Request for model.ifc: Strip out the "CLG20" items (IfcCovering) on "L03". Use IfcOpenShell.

First a look at what the model holds.

```python
import ifcopenshell
import ifcopenshell.util.element

model = ifcopenshell.open("model.ifc")
print(model.schema)
storey = next(s for s in model.by_type("IfcBuildingStorey") if s.Name == "L03")
coverings = [e for e in ifcopenshell.util.element.get_decomposition(storey) if e.is_a("IfcCovering")]
seen = {}
for e in coverings:
    element_type = ifcopenshell.util.element.get_type(e)
    name = element_type.Name if element_type not in (None, e) else None
    seen[name] = seen.get(name, 0) + 1
for name, count in sorted(seen.items(), key=str):
    print(count, "x", name)
```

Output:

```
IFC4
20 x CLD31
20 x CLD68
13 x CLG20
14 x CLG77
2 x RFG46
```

```python
import ifcopenshell
import ifcopenshell.api.root
import ifcopenshell.util.element

model = ifcopenshell.open("model.ifc")

storey = next(s for s in model.by_type("IfcBuildingStorey") if s.Name == "L03")
coverings = [e for e in ifcopenshell.util.element.get_decomposition(storey) if e.is_a("IfcCovering")]
targets = [e for e in coverings if (t := ifcopenshell.util.element.get_type(e)) not in (None, e) and t.Name == "CLG20"]

for e in targets:
    ifcopenshell.api.root.remove_product(model, product=e)
print(len(targets), "removed")

model.write("model_edited.ifc")
```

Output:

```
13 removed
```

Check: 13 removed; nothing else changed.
